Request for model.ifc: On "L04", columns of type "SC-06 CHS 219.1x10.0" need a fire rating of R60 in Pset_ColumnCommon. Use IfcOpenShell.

First a look at what the model holds.

```python
import ifcopenshell
import ifcopenshell.util.element

model = ifcopenshell.open("model.ifc")
print(model.schema)
storey = next(s for s in model.by_type("IfcBuildingStorey") if s.Name == "L04")
columns = [e for e in ifcopenshell.util.element.get_decomposition(storey) if e.is_a("IfcColumn")]
seen = {}
for e in columns:
    element_type = ifcopenshell.util.element.get_type(e)
    key = (element_type.Name if element_type != e and element_type else None, ifcopenshell.util.element.get_pset(e, "Pset_ColumnCommon", "FireRating"))
    seen[key] = seen.get(key, 0) + 1
for (name, value), count in sorted(seen.items(), key=str):
    print(count, "x", name, "|", value)
```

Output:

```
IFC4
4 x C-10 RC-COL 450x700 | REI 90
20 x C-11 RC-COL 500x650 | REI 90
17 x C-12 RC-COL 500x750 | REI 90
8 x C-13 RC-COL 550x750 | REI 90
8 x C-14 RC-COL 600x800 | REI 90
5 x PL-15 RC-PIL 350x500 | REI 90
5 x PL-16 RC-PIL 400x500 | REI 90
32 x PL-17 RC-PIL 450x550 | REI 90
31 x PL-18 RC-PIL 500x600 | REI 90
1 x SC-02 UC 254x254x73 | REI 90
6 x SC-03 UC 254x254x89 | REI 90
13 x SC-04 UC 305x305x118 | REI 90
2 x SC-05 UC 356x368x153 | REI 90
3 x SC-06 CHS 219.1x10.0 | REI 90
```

```python
import ifcopenshell
import ifcopenshell.api.pset
import ifcopenshell.util.element

model = ifcopenshell.open("model.ifc")

storey = next(s for s in model.by_type("IfcBuildingStorey") if s.Name == "L04")
columns = [e for e in ifcopenshell.util.element.get_decomposition(storey) if e.is_a("IfcColumn")]

count = 0
for e in columns:
    element_type = ifcopenshell.util.element.get_type(e)
    if element_type in (None, e) or element_type.Name != "SC-06 CHS 219.1x10.0":
        continue
    # add_pset returns the element's existing set when there is one.
    pset = ifcopenshell.api.pset.add_pset(model, product=e, name="Pset_ColumnCommon")
    ifcopenshell.api.pset.edit_pset(model, pset=pset, properties={"FireRating": "R60"})
    count += 1

print(count, "columns updated")

model.write("model_rev.ifc")
```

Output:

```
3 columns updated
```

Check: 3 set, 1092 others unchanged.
